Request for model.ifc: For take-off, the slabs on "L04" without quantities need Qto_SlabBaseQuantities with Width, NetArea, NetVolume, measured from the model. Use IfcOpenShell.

First a look at what the model holds.

```python
import ifcopenshell
import ifcopenshell.util.element
import ifcopenshell.util.unit

model = ifcopenshell.open("model.ifc")
print(model.schema)
for unit_type in ("LENGTHUNIT", "AREAUNIT", "VOLUMEUNIT"):
    print(unit_type, ifcopenshell.util.unit.calculate_unit_scale(model, unit_type))
storey = next(s for s in model.by_type("IfcBuildingStorey") if s.Name == "L04")
slabs = [e for e in ifcopenshell.util.element.get_decomposition(storey) if e.is_a("IfcSlab")]
for e in sorted(slabs, key=lambda e: e.id()):
    print(e.id(), e.is_a(), e.Name, list(ifcopenshell.util.element.get_psets(e, qtos_only=True)), sep=" | ")
```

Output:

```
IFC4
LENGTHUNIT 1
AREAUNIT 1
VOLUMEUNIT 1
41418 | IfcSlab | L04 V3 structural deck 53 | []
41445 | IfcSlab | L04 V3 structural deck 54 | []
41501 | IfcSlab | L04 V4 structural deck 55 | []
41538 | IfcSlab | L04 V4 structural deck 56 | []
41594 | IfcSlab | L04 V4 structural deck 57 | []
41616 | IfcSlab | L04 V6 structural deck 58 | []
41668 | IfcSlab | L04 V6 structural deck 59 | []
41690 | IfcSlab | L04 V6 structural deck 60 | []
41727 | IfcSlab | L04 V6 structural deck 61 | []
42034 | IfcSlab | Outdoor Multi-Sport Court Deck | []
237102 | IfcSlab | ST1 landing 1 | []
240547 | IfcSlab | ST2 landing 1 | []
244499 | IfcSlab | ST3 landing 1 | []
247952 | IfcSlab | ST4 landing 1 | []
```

```python
import ifcopenshell
import ifcopenshell.api.pset
import ifcopenshell.geom
import ifcopenshell.util.element
import ifcopenshell.util.shape
import ifcopenshell.util.unit

model = ifcopenshell.open("model.ifc")
unit_scale = ifcopenshell.util.unit.calculate_unit_scale(model)
area_scale = ifcopenshell.util.unit.calculate_unit_scale(model, "AREAUNIT")
volume_scale = ifcopenshell.util.unit.calculate_unit_scale(model, "VOLUMEUNIT")
settings = ifcopenshell.geom.settings()

storey = next(s for s in model.by_type("IfcBuildingStorey") if s.Name == "L04")
slabs = [e for e in ifcopenshell.util.element.get_decomposition(storey) if e.is_a("IfcSlab")]

for e in sorted(slabs, key=lambda e: e.id()):
    if ifcopenshell.util.element.get_psets(e, qtos_only=True, should_inherit=False):
        continue
    # Geometry comes back in metres, in the element's own axes.
    shape = ifcopenshell.geom.create_shape(settings, e)
    values = {
        "Width": ifcopenshell.util.shape.get_z(shape.geometry) / unit_scale,
        "NetArea": ifcopenshell.util.shape.get_footprint_area(shape.geometry) / area_scale,
        "NetVolume": ifcopenshell.util.shape.get_volume(shape.geometry) / volume_scale,
    }
    qto = ifcopenshell.api.pset.add_qto(model, product=e, name="Qto_SlabBaseQuantities")
    ifcopenshell.api.pset.edit_qto(model, qto=qto, properties=values)
    print(e.id(), {k: round(v, 3) for k, v in values.items()})

model.write("model_updated.ifc")
```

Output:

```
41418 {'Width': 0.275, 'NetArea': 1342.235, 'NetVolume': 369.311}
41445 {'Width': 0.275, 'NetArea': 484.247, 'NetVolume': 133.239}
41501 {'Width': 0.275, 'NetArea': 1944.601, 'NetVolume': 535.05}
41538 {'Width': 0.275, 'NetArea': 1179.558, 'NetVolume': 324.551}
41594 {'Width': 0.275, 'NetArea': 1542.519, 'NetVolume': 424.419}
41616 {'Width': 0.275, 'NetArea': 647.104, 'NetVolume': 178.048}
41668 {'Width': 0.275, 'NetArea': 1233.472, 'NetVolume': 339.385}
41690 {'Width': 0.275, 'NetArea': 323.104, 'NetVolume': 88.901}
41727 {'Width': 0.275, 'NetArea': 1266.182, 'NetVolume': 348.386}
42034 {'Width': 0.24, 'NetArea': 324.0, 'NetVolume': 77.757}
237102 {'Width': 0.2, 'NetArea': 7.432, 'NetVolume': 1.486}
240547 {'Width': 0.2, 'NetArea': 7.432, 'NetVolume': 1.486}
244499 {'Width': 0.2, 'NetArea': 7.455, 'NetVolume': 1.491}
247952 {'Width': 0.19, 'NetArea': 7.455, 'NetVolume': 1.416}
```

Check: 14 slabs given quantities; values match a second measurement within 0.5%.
